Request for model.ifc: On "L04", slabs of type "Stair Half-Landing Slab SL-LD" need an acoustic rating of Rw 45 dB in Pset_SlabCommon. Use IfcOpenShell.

First a look at what the model holds.

```python
import ifcopenshell
import ifcopenshell.util.element

model = ifcopenshell.open("model.ifc")
print(model.schema)
storey = next(s for s in model.by_type("IfcBuildingStorey") if s.Name == "L04")
slabs = [e for e in ifcopenshell.util.element.get_decomposition(storey) if e.is_a("IfcSlab")]
seen = {}
for e in slabs:
    element_type = ifcopenshell.util.element.get_type(e)
    key = (element_type.Name if element_type != e and element_type else None, ifcopenshell.util.element.get_pset(e, "Pset_SlabCommon", "AcousticRating"))
    seen[key] = seen.get(key, 0) + 1
for (name, value), count in sorted(seen.items(), key=str):
    print(count, "x", name, "|", value)
```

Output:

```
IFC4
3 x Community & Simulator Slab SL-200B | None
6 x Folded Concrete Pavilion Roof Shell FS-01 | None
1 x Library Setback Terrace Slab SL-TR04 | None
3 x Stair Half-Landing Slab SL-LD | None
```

```python
import ifcopenshell
import ifcopenshell.api.pset
import ifcopenshell.util.element

model = ifcopenshell.open("model.ifc")

storey = next(s for s in model.by_type("IfcBuildingStorey") if s.Name == "L04")
slabs = [e for e in ifcopenshell.util.element.get_decomposition(storey) if e.is_a("IfcSlab")]

count = 0
for e in slabs:
    element_type = ifcopenshell.util.element.get_type(e)
    if element_type in (None, e) or element_type.Name != "Stair Half-Landing Slab SL-LD":
        continue
    # add_pset returns the element's existing set when there is one.
    pset = ifcopenshell.api.pset.add_pset(model, product=e, name="Pset_SlabCommon")
    ifcopenshell.api.pset.edit_pset(model, pset=pset, properties={"AcousticRating": "Rw 45 dB"})
    count += 1

print(count, "slabs updated")

model.write("model_rev.ifc")
```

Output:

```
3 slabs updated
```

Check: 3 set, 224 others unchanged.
